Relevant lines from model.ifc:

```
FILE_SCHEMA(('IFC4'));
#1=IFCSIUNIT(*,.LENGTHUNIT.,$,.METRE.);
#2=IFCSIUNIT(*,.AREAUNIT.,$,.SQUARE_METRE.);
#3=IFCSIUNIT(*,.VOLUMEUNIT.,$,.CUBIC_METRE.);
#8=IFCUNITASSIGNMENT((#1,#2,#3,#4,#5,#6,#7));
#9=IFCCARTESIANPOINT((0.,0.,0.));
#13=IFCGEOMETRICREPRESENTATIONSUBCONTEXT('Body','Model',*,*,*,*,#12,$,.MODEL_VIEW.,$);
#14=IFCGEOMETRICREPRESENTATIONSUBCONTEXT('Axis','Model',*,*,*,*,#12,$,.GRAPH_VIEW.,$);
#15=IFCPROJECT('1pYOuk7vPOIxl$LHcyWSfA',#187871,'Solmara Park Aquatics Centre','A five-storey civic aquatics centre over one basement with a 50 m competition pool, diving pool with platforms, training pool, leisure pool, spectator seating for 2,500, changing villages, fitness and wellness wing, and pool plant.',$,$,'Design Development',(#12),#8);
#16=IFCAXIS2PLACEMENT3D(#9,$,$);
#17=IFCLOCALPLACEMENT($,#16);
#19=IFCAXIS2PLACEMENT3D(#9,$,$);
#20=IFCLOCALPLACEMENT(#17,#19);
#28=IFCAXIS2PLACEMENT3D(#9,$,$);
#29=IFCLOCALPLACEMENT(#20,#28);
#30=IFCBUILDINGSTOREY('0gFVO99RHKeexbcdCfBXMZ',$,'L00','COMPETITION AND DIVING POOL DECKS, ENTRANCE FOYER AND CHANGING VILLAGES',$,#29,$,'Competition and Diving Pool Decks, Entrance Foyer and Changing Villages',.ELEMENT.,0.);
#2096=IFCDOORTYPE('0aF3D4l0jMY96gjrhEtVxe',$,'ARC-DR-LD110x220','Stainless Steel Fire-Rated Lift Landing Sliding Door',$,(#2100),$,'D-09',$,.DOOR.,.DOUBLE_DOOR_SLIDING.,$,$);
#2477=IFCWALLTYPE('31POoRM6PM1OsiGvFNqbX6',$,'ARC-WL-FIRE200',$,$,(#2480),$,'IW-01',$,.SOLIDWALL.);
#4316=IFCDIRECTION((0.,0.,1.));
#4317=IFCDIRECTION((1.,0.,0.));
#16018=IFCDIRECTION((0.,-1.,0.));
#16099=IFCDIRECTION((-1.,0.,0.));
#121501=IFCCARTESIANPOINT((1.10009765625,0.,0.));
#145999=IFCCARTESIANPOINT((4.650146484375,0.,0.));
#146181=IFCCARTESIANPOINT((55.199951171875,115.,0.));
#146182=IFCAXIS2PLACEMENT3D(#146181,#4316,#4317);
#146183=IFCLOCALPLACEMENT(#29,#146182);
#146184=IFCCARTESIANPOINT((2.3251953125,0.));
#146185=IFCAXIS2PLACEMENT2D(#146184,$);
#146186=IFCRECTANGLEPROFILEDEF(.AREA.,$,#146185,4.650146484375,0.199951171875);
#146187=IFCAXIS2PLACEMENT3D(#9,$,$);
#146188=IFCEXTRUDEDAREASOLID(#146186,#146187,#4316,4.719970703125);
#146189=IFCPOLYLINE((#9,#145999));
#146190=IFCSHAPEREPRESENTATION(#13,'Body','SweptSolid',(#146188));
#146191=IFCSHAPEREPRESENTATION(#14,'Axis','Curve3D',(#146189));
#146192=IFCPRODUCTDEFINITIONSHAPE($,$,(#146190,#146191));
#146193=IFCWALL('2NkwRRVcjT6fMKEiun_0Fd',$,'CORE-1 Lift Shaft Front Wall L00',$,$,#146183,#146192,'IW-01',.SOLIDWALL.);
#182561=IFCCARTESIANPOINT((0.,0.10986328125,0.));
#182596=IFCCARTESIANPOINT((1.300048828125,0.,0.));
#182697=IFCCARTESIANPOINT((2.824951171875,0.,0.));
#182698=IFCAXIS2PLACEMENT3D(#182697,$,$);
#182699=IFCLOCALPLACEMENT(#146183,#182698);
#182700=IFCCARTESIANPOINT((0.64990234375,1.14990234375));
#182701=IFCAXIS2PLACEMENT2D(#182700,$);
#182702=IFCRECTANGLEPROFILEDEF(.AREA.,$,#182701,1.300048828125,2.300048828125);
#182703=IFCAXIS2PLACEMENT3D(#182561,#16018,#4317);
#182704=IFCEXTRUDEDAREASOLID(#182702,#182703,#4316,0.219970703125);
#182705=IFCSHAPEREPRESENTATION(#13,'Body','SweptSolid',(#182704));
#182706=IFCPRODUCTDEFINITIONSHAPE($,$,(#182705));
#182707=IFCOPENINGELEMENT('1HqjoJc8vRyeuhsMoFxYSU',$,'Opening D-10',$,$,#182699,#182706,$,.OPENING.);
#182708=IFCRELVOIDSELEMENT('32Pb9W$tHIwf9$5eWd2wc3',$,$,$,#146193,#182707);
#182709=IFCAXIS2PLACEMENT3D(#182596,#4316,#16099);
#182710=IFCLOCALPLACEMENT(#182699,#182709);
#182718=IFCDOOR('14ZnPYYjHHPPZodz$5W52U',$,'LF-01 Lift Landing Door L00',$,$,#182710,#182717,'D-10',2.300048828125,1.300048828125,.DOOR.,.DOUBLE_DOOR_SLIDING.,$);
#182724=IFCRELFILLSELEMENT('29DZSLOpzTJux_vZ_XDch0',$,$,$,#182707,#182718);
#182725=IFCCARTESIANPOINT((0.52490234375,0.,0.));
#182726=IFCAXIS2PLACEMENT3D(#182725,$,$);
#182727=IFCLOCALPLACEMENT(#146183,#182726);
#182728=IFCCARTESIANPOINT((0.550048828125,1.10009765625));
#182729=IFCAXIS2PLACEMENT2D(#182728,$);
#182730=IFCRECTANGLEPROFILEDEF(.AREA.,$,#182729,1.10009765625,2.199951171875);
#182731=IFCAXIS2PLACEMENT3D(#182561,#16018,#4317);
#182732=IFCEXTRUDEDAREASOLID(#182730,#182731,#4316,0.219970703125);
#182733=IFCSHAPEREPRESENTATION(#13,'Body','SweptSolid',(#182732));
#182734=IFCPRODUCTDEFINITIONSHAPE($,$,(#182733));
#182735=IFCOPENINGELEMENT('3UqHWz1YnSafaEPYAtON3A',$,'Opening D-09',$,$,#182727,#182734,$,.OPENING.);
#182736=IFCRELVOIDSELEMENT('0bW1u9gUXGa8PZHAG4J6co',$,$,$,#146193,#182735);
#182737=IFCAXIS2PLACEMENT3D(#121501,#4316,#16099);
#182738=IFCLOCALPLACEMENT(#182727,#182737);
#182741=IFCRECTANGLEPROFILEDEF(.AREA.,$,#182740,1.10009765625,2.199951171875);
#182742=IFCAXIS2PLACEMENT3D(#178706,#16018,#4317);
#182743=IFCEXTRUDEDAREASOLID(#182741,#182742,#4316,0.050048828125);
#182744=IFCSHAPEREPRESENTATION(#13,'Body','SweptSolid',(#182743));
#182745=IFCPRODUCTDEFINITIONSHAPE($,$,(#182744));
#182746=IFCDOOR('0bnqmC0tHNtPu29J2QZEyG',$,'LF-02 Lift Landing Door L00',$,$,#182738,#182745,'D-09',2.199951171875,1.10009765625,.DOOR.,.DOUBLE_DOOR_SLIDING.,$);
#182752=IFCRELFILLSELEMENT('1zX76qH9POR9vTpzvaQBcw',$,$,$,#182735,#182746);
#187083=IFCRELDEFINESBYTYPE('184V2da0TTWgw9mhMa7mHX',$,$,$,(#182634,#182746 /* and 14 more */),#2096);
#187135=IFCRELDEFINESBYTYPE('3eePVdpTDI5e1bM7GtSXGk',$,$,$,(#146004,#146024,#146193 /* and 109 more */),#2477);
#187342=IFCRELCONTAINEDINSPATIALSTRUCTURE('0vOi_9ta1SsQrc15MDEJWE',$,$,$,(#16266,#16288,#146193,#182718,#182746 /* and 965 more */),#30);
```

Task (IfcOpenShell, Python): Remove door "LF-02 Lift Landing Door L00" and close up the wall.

```python
import ifcopenshell
import ifcopenshell.api.feature
import ifcopenshell.api.root
import ifcopenshell.geom
import ifcopenshell.util.shape

model = ifcopenshell.open("model.ifc")
settings = ifcopenshell.geom.settings()


def volume(element):
    """Net volume in cubic metres, openings subtracted."""
    shape = ifcopenshell.geom.create_shape(settings, element)
    return ifcopenshell.util.shape.get_volume(shape.geometry)


door = model.by_guid("0bnqmC0tHNtPu29J2QZEyG")
opening = door.FillsVoids[0].RelatingOpeningElement
wall = opening.VoidsElements[0].RelatingBuildingElement
before = volume(wall)

ifcopenshell.api.root.remove_product(model, product=door)
ifcopenshell.api.feature.remove_feature(model, feature=opening)

after = volume(wall)

print(f"wall volume {before:.3f} -> {after:.3f} m3")

model.write("model-out.ifc")
```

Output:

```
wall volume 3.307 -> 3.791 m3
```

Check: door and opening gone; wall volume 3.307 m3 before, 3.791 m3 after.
